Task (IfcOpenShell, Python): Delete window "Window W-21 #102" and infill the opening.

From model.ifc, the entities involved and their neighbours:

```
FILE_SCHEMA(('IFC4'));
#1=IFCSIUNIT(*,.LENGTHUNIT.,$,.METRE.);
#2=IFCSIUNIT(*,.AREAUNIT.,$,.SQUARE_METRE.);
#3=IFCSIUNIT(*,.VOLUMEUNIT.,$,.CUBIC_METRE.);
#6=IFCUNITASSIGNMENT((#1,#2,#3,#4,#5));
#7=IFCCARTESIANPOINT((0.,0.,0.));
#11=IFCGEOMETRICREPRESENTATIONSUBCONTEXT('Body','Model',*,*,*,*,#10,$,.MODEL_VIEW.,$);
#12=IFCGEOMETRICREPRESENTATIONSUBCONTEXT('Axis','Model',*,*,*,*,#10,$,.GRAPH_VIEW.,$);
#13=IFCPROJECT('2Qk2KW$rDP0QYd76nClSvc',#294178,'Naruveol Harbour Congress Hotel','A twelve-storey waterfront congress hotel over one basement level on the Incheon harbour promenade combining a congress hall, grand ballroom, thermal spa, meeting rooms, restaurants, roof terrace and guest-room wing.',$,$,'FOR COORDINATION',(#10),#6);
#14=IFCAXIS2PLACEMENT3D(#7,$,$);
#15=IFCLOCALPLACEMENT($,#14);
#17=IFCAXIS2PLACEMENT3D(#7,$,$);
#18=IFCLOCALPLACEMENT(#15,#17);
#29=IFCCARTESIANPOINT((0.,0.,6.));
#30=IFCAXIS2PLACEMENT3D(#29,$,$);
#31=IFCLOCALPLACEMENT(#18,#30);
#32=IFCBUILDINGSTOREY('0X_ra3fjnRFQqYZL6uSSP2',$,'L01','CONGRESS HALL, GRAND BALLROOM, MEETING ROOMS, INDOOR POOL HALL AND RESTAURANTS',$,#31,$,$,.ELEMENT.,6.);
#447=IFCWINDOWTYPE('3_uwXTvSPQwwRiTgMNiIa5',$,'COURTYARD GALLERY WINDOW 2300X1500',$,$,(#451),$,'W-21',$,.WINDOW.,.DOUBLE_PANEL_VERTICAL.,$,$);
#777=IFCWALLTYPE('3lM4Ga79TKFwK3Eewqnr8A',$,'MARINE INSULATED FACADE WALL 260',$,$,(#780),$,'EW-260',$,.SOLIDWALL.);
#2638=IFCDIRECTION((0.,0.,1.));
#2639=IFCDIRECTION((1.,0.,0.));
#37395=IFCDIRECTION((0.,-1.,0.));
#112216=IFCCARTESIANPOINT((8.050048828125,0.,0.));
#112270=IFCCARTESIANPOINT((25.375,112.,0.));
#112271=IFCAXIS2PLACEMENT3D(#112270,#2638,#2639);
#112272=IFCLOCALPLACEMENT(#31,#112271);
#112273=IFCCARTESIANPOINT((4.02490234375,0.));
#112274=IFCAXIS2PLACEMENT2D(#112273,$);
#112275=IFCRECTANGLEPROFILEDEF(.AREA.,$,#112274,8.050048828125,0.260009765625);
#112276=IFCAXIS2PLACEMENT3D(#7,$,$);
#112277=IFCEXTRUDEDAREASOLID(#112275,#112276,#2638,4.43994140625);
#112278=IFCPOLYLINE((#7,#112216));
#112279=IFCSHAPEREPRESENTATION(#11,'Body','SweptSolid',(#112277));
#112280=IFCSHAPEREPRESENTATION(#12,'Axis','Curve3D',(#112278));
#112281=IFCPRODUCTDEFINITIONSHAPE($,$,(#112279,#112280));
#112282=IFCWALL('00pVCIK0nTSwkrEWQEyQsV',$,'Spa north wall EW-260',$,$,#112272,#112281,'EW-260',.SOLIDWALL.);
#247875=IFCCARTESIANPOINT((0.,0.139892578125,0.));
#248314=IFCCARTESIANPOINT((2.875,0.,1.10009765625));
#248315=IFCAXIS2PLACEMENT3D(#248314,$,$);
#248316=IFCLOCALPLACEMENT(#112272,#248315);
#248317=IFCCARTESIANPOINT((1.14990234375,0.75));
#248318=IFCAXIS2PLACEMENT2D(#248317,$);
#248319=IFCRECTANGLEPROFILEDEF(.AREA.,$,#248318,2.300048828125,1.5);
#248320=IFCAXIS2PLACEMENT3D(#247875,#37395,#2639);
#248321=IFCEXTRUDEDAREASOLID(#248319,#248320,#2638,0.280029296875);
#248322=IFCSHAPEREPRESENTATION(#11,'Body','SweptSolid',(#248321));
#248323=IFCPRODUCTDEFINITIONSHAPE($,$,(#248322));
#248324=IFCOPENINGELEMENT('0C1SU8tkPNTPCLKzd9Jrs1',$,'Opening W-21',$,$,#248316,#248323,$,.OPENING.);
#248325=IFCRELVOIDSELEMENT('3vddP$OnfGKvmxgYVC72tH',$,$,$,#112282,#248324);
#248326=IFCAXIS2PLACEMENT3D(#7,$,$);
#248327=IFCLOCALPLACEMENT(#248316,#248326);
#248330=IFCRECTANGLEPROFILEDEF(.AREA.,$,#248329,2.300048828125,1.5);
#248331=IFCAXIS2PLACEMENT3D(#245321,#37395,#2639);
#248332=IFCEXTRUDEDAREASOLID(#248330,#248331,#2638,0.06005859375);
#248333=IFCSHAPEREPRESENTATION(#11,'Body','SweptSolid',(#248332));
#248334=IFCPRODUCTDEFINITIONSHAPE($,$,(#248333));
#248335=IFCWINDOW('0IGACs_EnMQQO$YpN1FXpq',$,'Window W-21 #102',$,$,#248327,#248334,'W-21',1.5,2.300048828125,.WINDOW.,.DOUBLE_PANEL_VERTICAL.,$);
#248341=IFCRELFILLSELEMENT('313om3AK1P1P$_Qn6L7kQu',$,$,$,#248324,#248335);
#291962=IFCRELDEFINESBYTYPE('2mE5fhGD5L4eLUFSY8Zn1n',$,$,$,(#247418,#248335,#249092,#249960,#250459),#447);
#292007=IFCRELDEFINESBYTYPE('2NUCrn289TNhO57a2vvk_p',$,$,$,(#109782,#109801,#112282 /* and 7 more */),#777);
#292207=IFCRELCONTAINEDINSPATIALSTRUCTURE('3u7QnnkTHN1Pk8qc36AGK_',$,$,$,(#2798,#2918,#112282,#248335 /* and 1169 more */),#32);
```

```python
import ifcopenshell
import ifcopenshell.api.feature
import ifcopenshell.api.root
import ifcopenshell.geom
import ifcopenshell.util.shape

model = ifcopenshell.open("model.ifc")
settings = ifcopenshell.geom.settings()


def volume(element):
    """Net volume in cubic metres, openings subtracted."""
    shape = ifcopenshell.geom.create_shape(settings, element)
    return ifcopenshell.util.shape.get_volume(shape.geometry)


window = model.by_guid("0IGACs_EnMQQO$YpN1FXpq")
opening = window.FillsVoids[0].RelatingOpeningElement
wall = opening.VoidsElements[0].RelatingBuildingElement
before = volume(wall)

ifcopenshell.api.root.remove_product(model, product=window)
ifcopenshell.api.feature.remove_feature(model, feature=opening)

after = volume(wall)

print(f"wall volume {before:.3f} -> {after:.3f} m3")

model.write("model_edited.ifc")
```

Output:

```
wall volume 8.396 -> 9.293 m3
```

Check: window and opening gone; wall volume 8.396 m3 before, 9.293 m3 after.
